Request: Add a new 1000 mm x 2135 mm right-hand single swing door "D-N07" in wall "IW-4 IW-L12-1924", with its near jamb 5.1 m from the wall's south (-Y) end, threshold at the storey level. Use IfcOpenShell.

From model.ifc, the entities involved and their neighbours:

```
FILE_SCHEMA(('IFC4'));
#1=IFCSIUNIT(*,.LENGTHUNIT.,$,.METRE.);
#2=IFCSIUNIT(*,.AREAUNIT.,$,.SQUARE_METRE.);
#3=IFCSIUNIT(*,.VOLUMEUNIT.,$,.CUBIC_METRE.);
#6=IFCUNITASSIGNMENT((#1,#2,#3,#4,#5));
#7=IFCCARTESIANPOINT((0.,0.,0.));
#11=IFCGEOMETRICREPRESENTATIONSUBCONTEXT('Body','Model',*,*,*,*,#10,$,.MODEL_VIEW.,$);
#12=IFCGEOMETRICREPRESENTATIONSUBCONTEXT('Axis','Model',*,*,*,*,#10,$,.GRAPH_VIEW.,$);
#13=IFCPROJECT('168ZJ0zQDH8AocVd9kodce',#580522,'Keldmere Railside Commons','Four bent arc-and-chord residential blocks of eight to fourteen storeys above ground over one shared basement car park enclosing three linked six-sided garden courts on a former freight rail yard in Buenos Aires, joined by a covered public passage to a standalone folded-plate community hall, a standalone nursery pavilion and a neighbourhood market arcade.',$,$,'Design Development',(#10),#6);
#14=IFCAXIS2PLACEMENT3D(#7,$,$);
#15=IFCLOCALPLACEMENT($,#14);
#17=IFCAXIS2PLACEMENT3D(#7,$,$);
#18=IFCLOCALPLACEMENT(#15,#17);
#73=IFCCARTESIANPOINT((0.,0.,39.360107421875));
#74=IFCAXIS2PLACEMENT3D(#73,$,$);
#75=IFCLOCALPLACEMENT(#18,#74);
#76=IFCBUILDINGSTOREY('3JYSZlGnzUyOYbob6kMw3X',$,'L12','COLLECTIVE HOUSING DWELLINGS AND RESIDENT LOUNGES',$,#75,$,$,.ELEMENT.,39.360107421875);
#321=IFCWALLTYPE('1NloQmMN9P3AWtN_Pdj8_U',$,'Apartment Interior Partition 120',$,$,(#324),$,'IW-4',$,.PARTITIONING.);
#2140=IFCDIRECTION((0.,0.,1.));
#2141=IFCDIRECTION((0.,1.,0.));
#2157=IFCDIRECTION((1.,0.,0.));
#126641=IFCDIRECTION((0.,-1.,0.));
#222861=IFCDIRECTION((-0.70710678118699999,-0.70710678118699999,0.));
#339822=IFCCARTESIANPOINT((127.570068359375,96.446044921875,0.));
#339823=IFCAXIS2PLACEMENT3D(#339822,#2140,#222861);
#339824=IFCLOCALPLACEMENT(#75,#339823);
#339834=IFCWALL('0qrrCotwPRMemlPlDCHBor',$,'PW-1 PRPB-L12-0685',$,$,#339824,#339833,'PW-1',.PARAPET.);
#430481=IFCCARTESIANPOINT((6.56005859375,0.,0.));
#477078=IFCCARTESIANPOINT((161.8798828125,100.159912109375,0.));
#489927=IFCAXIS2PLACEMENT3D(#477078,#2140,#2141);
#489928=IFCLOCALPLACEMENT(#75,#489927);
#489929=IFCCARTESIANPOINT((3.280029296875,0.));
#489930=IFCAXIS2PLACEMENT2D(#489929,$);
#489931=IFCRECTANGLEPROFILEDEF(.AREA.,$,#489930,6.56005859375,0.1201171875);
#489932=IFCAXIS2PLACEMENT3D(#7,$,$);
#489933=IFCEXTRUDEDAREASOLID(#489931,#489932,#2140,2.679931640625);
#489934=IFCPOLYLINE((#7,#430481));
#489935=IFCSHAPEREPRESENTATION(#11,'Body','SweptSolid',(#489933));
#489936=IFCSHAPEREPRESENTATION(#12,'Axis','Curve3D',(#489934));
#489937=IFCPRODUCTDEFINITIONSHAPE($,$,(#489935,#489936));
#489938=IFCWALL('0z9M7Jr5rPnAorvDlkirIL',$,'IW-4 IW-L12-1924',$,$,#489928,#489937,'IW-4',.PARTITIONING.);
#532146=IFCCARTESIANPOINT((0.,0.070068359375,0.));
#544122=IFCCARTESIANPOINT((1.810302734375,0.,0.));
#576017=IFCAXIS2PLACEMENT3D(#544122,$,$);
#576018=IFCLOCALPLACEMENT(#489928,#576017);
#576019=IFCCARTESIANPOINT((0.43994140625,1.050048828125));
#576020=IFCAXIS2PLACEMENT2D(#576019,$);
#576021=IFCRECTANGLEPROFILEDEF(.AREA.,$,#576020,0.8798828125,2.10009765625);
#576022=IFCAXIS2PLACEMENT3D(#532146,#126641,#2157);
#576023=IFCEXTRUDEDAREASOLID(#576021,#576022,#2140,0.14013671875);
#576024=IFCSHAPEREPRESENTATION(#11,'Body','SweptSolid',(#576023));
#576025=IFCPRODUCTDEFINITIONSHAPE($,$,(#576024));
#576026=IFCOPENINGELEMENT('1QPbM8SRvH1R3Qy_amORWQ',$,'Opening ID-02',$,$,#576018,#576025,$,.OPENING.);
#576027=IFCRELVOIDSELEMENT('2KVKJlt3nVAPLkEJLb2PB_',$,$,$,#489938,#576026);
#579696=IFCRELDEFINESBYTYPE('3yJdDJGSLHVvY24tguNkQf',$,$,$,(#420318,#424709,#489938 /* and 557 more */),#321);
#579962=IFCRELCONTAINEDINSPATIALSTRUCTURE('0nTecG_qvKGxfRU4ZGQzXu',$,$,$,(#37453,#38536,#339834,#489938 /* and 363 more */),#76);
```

```python
import numpy as np
import ifcopenshell
import ifcopenshell.api.feature
import ifcopenshell.api.geometry
import ifcopenshell.api.root
import ifcopenshell.api.spatial
import ifcopenshell.geom
import ifcopenshell.util.element
import ifcopenshell.util.placement
import ifcopenshell.util.representation
import ifcopenshell.util.shape
import ifcopenshell.util.unit

model = ifcopenshell.open("model.ifc")
unit_scale = ifcopenshell.util.unit.calculate_unit_scale(model)
settings = ifcopenshell.geom.settings()


def volume(element):
    """Net volume in cubic metres, openings subtracted."""
    shape = ifcopenshell.geom.create_shape(settings, element)
    return ifcopenshell.util.shape.get_volume(shape.geometry)


wall = model.by_id(489938)
storey = ifcopenshell.util.element.get_container(wall, ifc_class="IfcBuildingStorey")
context = ifcopenshell.util.representation.get_context(model, "Model", "Body", "MODEL_VIEW")
before = volume(wall)

width, height, from_end, sill = 1, 2.135, 5.1, 0.0  # metres

# The wall runs along its own X axis, and the end named is its -X end.
wall_shape = ifcopenshell.geom.create_shape(settings, wall)
x, y, z = ifcopenshell.util.shape.get_vertices(wall_shape.geometry).T
start = x.min() + from_end
face, thickness = float(y.min()), float(y.max() - y.min())
wall_matrix = ifcopenshell.util.placement.get_local_placement(wall.ObjectPlacement)
level = ifcopenshell.util.placement.get_local_placement(storey.ObjectPlacement)[2, 3]


def in_wall(x, y):
    """Placement at x, y metres in the wall's axes, at sill height."""
    matrix = wall_matrix.copy()
    matrix[:, 3] = wall_matrix @ np.array([x / unit_scale, y / unit_scale, 0.0, 1.0])
    matrix[2, 3] = level + sill / unit_scale
    return matrix


# Opening: a box that overshoots both wall faces by 50 mm.
opening = ifcopenshell.api.root.create_entity(model, ifc_class="IfcOpeningElement", predefined_type="OPENING")
box = ifcopenshell.api.geometry.add_wall_representation(
    model, context=context, length=width, height=height, thickness=thickness + 0.1
)
ifcopenshell.api.geometry.assign_representation(model, product=opening, representation=box)
ifcopenshell.api.geometry.edit_object_placement(model, product=opening, matrix=in_wall(start, face - 0.05), is_si=False)
ifcopenshell.api.feature.add_feature(model, feature=opening, element=wall)

door = ifcopenshell.api.root.create_entity(model, ifc_class="IfcDoor", name="D-N07", predefined_type="DOOR")
door.OverallWidth, door.OverallHeight = width / unit_scale, height / unit_scale
door.OperationType = "SINGLE_SWING_RIGHT"
body = ifcopenshell.api.geometry.add_door_representation(
    model,
    context=context,
    overall_width=door.OverallWidth,
    overall_height=door.OverallHeight,
    operation_type="SINGLE_SWING_RIGHT",
    lining_properties={"LiningDepth": thickness / unit_scale, "ThresholdDepth": thickness / unit_scale},
)
ifcopenshell.api.geometry.assign_representation(model, product=door, representation=body)
ifcopenshell.api.spatial.assign_container(model, products=[door], relating_structure=storey)
ifcopenshell.api.feature.add_filling(model, opening=opening, element=door)

# The lining spans the wall, so the door starts at the wall face.
ifcopenshell.api.geometry.edit_object_placement(model, product=door, matrix=in_wall(start, face), is_si=False)

after = volume(wall)

print(f"wall volume {before:.3f} -> {after:.3f} m3")

model.write("model_v2.ifc")
```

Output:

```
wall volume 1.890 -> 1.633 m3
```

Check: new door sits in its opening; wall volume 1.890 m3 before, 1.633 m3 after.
